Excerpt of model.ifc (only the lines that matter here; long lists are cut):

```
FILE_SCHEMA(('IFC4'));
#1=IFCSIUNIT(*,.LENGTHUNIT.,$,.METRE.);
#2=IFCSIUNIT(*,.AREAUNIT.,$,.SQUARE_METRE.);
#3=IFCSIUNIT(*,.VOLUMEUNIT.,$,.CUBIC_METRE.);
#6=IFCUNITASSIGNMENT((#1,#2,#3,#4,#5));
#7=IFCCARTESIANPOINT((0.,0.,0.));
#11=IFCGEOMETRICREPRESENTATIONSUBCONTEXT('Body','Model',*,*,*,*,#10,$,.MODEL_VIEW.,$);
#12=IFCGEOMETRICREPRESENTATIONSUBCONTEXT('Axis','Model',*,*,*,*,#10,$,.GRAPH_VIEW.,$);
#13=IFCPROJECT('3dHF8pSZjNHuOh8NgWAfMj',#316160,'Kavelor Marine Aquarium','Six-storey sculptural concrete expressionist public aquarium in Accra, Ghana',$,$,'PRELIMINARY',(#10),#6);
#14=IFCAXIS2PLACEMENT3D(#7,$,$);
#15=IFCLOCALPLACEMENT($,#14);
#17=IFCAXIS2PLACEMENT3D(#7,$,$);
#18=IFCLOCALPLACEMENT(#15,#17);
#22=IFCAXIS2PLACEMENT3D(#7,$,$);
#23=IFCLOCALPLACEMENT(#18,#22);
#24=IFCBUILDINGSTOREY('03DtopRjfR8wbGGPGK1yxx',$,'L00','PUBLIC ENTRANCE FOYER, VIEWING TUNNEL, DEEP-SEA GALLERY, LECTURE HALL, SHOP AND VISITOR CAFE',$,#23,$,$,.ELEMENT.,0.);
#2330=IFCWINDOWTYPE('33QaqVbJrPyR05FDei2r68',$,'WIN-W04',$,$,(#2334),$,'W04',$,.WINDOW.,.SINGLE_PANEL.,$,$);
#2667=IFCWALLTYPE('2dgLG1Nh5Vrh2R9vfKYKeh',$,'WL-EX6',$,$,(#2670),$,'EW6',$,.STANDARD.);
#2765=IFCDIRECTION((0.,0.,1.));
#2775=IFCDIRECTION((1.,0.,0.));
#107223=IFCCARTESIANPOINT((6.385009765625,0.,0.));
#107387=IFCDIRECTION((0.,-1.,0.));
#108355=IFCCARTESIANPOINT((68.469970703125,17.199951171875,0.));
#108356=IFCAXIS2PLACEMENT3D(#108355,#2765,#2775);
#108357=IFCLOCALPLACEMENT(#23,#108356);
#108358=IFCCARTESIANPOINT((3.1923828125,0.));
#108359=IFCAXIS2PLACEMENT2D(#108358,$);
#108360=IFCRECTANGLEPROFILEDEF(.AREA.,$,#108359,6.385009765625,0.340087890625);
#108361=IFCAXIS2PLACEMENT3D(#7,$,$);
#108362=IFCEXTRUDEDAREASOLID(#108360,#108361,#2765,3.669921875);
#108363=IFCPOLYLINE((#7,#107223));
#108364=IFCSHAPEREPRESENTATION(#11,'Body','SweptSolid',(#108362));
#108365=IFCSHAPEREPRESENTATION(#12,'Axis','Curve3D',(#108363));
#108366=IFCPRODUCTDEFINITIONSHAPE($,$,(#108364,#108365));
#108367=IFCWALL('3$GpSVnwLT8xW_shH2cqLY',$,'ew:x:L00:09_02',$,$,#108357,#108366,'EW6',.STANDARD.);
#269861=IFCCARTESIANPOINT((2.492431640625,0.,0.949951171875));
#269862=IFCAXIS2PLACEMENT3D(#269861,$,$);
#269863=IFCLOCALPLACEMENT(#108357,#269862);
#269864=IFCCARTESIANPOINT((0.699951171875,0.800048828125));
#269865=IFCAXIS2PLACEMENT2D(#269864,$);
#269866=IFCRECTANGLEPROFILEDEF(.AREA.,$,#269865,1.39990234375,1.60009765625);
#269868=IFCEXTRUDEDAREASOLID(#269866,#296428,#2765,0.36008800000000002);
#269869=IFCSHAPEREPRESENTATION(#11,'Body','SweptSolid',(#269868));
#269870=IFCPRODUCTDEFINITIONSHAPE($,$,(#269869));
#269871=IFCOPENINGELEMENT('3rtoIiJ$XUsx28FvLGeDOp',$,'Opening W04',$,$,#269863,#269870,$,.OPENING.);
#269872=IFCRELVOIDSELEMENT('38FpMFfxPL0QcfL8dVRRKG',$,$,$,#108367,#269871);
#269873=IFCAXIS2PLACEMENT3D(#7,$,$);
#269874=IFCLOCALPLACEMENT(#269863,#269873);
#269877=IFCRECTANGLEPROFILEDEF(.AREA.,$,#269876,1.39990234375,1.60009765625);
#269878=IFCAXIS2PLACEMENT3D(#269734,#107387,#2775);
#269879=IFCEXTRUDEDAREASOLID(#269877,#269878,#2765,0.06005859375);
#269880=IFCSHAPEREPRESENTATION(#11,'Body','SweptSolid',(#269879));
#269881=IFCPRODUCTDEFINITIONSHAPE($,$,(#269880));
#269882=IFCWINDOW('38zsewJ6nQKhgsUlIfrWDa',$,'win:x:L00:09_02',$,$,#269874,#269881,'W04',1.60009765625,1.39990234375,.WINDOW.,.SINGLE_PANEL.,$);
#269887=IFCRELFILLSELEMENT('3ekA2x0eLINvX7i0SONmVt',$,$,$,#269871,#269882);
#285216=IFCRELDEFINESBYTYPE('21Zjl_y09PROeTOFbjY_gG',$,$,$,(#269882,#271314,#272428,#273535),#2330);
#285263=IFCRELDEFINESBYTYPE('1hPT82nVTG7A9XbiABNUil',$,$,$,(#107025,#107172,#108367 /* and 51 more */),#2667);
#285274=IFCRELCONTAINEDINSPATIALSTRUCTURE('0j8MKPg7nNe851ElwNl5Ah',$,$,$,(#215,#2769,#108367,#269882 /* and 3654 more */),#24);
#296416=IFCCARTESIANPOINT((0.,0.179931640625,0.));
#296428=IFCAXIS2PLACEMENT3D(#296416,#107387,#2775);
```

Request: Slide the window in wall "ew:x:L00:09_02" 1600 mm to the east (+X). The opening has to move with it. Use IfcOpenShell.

```python
import ifcopenshell
import ifcopenshell.api.geometry
import ifcopenshell.util.placement
import ifcopenshell.util.unit

model = ifcopenshell.open("model.ifc")
unit_scale = ifcopenshell.util.unit.calculate_unit_scale(model)

window = model.by_guid("38zsewJ6nQKhgsUlIfrWDa")
opening = window.FillsVoids[0].RelatingOpeningElement
wall = opening.VoidsElements[0].RelatingBuildingElement

wall_matrix = ifcopenshell.util.placement.get_local_placement(wall.ObjectPlacement)
shift = wall_matrix[:3, 0] * 1.6 / unit_scale
before = ifcopenshell.util.placement.get_local_placement(window.ObjectPlacement)[:3, 3].copy()

# The window is placed relative to its opening, so it follows when the opening moves.
matrix = ifcopenshell.util.placement.get_local_placement(opening.ObjectPlacement)
matrix[:3, 3] += shift
ifcopenshell.api.geometry.edit_object_placement(
    model, product=opening, matrix=matrix, is_si=False, should_transform_children=True
)

after = ifcopenshell.util.placement.get_local_placement(window.ObjectPlacement)[:3, 3]
print("window moved by", (after - before).round(3) + 0.0)

model.write("model_rev.ifc")
```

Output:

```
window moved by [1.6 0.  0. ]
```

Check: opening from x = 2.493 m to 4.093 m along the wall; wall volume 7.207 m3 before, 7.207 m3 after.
